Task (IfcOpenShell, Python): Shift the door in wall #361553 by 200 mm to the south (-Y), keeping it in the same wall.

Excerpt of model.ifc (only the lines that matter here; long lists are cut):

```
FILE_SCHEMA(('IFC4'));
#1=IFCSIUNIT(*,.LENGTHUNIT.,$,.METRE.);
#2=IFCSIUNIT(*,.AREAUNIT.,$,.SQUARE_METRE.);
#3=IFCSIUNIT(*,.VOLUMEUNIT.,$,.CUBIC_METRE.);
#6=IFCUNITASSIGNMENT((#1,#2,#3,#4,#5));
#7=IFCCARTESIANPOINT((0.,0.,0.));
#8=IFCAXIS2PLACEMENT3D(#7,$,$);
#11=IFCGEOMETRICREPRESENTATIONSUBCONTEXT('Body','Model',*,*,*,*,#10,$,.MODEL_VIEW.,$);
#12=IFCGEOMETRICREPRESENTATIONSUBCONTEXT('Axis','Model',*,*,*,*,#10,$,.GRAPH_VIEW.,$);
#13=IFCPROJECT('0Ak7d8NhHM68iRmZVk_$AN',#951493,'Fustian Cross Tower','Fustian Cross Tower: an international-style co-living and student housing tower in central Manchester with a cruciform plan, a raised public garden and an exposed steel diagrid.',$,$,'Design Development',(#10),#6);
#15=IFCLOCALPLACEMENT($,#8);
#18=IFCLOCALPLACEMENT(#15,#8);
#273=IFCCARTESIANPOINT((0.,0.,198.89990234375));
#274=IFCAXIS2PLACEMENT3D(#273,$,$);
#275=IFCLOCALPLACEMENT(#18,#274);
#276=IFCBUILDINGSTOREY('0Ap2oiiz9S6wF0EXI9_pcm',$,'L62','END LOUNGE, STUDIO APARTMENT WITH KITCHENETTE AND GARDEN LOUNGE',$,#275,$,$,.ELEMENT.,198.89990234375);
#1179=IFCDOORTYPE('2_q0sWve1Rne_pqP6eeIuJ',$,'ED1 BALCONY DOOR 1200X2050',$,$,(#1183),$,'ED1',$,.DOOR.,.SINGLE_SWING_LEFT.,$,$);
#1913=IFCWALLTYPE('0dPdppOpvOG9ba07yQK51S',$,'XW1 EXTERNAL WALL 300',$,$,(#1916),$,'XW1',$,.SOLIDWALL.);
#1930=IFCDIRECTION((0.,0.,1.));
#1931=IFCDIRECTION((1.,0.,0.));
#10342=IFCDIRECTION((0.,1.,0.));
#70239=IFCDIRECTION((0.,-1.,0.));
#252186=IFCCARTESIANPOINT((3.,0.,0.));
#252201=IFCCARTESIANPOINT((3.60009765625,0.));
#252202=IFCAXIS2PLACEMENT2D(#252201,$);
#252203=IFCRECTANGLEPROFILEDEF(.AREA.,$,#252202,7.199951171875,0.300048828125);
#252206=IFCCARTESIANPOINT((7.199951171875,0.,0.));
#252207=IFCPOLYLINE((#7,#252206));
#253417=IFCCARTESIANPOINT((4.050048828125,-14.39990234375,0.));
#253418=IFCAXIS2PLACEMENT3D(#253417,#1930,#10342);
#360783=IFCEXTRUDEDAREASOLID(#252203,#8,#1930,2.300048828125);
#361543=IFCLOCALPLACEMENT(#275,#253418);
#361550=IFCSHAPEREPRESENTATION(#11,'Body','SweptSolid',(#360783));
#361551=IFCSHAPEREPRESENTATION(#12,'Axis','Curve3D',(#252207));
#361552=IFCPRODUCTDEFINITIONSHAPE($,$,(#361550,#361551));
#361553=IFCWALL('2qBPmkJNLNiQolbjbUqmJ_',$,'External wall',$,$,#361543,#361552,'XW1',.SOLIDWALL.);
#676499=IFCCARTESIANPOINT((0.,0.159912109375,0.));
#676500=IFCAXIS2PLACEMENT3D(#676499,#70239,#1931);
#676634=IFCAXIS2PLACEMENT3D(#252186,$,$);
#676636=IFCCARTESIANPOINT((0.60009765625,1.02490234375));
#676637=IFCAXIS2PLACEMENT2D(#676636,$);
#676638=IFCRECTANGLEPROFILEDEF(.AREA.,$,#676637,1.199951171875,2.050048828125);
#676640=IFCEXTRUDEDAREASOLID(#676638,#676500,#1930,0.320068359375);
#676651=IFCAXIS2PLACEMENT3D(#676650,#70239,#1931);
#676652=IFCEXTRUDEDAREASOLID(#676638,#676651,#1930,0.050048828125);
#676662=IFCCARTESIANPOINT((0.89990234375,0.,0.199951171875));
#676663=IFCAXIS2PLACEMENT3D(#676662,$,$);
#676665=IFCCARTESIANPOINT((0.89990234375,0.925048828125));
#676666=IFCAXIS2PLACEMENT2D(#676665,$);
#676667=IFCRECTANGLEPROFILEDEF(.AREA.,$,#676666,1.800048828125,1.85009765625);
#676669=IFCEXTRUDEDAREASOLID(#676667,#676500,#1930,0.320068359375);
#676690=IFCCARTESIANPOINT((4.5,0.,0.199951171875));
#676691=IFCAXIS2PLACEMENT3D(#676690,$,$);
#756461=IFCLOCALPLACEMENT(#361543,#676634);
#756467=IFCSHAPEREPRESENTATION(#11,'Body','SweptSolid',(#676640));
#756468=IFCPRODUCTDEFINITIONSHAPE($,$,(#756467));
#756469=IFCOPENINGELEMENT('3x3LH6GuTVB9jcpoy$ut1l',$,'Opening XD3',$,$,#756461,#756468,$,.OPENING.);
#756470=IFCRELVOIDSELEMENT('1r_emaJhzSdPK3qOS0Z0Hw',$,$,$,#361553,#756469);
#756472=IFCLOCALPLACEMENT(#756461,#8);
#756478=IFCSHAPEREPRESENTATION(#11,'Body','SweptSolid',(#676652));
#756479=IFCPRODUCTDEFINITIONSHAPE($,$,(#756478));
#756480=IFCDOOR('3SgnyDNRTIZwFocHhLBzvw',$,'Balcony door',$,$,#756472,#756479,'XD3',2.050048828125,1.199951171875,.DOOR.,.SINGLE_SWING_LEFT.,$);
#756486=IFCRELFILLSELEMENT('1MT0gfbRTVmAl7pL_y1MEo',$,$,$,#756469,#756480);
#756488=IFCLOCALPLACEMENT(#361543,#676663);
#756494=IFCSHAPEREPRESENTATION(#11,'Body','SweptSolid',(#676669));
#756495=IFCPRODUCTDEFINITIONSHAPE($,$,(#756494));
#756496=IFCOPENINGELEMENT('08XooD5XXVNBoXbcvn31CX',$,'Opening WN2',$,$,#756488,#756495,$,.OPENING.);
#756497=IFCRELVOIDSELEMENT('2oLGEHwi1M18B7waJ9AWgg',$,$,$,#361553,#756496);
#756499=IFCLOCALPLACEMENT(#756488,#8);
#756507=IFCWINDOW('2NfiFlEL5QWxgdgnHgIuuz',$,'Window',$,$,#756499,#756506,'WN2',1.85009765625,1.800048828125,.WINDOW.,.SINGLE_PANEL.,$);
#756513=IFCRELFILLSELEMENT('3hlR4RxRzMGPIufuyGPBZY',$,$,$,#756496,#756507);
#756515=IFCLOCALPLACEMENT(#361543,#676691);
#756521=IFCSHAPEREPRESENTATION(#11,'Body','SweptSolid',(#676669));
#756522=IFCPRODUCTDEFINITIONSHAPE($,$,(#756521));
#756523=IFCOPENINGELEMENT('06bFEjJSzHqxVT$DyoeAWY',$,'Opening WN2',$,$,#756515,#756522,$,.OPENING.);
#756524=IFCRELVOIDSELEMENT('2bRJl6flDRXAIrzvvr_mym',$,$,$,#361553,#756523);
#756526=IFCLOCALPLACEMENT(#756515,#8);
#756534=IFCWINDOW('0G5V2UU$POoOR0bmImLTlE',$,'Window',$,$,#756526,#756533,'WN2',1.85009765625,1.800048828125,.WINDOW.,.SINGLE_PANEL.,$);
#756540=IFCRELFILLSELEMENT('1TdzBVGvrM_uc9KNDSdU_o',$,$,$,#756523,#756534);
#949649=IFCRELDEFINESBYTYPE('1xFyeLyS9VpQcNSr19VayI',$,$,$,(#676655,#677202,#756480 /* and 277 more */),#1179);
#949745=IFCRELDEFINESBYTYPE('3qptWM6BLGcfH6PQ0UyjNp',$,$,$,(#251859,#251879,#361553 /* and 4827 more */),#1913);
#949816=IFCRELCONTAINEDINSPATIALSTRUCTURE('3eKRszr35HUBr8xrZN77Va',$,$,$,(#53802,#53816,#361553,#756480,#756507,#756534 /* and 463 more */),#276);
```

```python
import ifcopenshell
import ifcopenshell.api.geometry
import ifcopenshell.util.placement

model = ifcopenshell.open("model.ifc")

door = model.by_id(756480)
opening = door.FillsVoids[0].RelatingOpeningElement
wall = opening.VoidsElements[0].RelatingBuildingElement

wall_matrix = ifcopenshell.util.placement.get_local_placement(wall.ObjectPlacement)
shift = wall_matrix[:3, 0] * -0.2
before = ifcopenshell.util.placement.get_local_placement(door.ObjectPlacement)[:3, 3].copy()

# The door is placed relative to its opening, so it follows when the opening moves.
matrix = ifcopenshell.util.placement.get_local_placement(opening.ObjectPlacement)
matrix[:3, 3] += shift
ifcopenshell.api.geometry.edit_object_placement(
    model, product=opening, matrix=matrix, is_si=False, should_transform_children=True
)

after = ifcopenshell.util.placement.get_local_placement(door.ObjectPlacement)[:3, 3]
print("door moved by", (after - before).round(3) + 0.0)

model.write("model-out.ifc")
```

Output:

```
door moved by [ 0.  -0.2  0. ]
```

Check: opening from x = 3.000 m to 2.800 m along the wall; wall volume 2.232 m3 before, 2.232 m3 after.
